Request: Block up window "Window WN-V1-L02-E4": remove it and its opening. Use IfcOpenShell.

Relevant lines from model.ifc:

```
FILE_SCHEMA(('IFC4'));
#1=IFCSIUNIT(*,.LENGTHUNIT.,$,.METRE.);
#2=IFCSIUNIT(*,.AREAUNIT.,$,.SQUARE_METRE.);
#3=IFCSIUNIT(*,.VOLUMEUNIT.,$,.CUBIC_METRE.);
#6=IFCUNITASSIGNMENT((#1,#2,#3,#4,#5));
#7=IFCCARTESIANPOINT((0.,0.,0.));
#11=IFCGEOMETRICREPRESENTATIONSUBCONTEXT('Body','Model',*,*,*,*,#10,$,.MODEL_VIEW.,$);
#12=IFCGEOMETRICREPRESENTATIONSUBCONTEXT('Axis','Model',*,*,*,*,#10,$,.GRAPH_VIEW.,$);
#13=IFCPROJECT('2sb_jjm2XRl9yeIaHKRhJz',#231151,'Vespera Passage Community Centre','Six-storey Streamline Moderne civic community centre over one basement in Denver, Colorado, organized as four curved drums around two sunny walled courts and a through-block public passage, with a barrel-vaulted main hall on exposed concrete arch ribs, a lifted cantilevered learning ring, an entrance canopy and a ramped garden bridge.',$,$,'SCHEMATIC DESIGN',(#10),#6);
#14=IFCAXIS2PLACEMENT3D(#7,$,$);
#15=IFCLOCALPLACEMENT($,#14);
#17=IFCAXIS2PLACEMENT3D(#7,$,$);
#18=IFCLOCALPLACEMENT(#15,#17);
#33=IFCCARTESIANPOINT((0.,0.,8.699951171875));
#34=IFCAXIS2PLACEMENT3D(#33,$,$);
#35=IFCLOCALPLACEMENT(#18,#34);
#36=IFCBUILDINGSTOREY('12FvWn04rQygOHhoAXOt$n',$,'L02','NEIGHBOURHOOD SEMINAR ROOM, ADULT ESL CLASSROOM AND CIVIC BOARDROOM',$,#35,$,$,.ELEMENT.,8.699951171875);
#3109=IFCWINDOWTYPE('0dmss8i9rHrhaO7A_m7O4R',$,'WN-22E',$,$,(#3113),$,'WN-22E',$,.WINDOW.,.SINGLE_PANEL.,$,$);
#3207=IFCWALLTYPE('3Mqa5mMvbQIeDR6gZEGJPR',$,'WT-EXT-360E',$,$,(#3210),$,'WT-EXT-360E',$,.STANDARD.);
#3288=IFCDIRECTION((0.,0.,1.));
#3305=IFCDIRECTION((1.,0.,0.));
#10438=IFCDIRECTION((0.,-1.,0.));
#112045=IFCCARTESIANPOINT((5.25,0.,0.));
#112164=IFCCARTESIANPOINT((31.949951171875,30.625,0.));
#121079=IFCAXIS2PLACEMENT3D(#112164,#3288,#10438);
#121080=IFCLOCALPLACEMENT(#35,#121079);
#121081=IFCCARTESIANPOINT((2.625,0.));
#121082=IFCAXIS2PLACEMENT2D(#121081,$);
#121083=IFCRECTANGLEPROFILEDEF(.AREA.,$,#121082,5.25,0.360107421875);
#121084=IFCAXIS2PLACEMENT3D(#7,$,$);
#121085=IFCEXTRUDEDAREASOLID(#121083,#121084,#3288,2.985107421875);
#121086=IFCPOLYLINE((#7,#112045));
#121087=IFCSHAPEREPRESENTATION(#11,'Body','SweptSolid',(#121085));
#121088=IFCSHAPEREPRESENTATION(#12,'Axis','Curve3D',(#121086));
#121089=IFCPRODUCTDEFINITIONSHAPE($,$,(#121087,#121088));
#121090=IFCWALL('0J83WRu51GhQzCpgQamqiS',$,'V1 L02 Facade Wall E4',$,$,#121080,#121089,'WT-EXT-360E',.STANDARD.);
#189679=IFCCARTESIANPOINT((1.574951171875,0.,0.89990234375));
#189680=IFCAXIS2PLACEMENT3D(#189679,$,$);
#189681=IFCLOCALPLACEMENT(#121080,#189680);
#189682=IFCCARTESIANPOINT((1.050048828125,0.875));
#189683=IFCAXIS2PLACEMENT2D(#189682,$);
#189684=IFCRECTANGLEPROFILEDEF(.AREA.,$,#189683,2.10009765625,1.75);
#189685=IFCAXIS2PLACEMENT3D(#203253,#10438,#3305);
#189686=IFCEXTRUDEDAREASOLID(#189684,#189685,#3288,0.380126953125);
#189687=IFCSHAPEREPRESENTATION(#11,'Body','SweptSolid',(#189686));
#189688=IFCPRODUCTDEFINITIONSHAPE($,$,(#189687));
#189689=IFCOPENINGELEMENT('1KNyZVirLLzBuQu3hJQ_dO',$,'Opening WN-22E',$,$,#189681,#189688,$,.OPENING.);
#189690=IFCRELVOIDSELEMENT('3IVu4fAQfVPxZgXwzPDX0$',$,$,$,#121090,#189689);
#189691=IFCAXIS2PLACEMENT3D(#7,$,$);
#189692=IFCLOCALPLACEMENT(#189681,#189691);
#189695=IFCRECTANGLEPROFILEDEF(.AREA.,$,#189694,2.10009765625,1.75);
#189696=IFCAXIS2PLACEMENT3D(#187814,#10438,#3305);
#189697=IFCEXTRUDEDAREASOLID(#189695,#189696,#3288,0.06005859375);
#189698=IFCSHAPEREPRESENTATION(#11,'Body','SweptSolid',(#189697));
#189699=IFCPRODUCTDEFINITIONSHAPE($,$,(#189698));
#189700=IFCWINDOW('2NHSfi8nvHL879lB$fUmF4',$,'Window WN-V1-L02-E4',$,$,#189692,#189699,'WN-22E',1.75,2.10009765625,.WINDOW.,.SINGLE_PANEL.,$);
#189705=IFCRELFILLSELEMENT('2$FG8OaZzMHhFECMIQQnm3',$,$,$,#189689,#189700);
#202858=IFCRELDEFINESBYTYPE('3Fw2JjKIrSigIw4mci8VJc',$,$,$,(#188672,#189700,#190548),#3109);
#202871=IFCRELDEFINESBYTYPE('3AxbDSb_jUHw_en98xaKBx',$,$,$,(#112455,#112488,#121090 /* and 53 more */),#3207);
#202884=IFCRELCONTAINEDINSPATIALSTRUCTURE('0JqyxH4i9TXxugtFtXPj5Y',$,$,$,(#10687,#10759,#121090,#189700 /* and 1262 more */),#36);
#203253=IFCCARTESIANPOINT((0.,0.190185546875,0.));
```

```python
import ifcopenshell
import ifcopenshell.api.feature
import ifcopenshell.api.root
import ifcopenshell.geom
import ifcopenshell.util.shape

model = ifcopenshell.open("model.ifc")
settings = ifcopenshell.geom.settings()


def volume(element):
    """Net volume in cubic metres, openings subtracted."""
    shape = ifcopenshell.geom.create_shape(settings, element)
    return ifcopenshell.util.shape.get_volume(shape.geometry)


window = model.by_guid("2NHSfi8nvHL879lB$fUmF4")
opening = window.FillsVoids[0].RelatingOpeningElement
wall = opening.VoidsElements[0].RelatingBuildingElement
before = volume(wall)

ifcopenshell.api.root.remove_product(model, product=window)
ifcopenshell.api.feature.remove_feature(model, feature=opening)

after = volume(wall)

print(f"wall volume {before:.3f} -> {after:.3f} m3")

model.write("model_edited.ifc")
```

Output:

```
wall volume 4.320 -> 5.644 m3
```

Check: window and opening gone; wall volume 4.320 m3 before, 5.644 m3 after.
